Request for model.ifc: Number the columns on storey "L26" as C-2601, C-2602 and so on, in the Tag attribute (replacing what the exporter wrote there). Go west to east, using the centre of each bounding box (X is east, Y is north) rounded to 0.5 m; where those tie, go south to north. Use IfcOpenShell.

First a look at what the model holds.

```python
import ifcopenshell
import ifcopenshell.util.element
import ifcopenshell.util.placement

model = ifcopenshell.open("model.ifc")
print(model.schema)
storey = next(s for s in model.by_type("IfcBuildingStorey") if s.Name == "L26")
columns = [e for e in ifcopenshell.util.element.get_decomposition(storey) if e.is_a("IfcColumn")]
for e in sorted(columns, key=lambda e: e.id()):
    origin = ifcopenshell.util.placement.get_local_placement(e.ObjectPlacement)[:3, 3]
    print(e.id(), e.Tag, e.Name, origin.round(2) + 0.0, sep=" | ")
```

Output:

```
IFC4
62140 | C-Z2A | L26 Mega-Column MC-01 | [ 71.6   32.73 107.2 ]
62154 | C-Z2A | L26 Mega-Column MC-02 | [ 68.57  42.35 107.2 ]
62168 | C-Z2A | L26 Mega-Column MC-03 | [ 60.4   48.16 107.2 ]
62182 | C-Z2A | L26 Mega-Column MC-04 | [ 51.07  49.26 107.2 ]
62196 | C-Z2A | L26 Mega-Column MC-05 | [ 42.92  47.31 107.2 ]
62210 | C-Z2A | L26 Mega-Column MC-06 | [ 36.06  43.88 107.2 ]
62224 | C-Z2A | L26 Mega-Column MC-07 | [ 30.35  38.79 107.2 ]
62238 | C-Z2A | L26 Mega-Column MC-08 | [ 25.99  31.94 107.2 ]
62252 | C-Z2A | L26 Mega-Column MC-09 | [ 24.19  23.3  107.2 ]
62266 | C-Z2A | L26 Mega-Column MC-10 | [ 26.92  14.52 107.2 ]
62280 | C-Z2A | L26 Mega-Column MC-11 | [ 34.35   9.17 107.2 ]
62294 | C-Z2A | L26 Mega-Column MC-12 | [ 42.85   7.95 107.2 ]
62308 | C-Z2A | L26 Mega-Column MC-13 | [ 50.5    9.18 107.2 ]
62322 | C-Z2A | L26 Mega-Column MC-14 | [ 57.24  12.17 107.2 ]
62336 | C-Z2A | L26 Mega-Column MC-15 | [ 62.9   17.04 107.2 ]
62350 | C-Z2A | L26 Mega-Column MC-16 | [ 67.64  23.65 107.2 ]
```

```python
import ifcopenshell
import ifcopenshell.geom
import ifcopenshell.util.element
import ifcopenshell.util.shape

model = ifcopenshell.open("model.ifc")
settings = ifcopenshell.geom.settings()
settings.set("use-world-coords", True)


def centre(element):
    shape = ifcopenshell.geom.create_shape(settings, element)
    return ifcopenshell.util.shape.get_bbox_centroid(shape.geometry)


storey = next(s for s in model.by_type("IfcBuildingStorey") if s.Name == "L26")
columns = [e for e in ifcopenshell.util.element.get_decomposition(storey) if e.is_a("IfcColumn")]

# Insertion points can sit at a corner or the storey origin, so sort by the geometry (in metres).
centres = {e: centre(e) for e in columns}
columns.sort(key=lambda e: (round(centres[e][0] / 0.5), centres[e][1]))

for i, e in enumerate(columns, start=1):
    number = f"C-26{i:02d}"
    e.Tag = number
    print(e.id(), number)

model.write("model_rev.ifc")
```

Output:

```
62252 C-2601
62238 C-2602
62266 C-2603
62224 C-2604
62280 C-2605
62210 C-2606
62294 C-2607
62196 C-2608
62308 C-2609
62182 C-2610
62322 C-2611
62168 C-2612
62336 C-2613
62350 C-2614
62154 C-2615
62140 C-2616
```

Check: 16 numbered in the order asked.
